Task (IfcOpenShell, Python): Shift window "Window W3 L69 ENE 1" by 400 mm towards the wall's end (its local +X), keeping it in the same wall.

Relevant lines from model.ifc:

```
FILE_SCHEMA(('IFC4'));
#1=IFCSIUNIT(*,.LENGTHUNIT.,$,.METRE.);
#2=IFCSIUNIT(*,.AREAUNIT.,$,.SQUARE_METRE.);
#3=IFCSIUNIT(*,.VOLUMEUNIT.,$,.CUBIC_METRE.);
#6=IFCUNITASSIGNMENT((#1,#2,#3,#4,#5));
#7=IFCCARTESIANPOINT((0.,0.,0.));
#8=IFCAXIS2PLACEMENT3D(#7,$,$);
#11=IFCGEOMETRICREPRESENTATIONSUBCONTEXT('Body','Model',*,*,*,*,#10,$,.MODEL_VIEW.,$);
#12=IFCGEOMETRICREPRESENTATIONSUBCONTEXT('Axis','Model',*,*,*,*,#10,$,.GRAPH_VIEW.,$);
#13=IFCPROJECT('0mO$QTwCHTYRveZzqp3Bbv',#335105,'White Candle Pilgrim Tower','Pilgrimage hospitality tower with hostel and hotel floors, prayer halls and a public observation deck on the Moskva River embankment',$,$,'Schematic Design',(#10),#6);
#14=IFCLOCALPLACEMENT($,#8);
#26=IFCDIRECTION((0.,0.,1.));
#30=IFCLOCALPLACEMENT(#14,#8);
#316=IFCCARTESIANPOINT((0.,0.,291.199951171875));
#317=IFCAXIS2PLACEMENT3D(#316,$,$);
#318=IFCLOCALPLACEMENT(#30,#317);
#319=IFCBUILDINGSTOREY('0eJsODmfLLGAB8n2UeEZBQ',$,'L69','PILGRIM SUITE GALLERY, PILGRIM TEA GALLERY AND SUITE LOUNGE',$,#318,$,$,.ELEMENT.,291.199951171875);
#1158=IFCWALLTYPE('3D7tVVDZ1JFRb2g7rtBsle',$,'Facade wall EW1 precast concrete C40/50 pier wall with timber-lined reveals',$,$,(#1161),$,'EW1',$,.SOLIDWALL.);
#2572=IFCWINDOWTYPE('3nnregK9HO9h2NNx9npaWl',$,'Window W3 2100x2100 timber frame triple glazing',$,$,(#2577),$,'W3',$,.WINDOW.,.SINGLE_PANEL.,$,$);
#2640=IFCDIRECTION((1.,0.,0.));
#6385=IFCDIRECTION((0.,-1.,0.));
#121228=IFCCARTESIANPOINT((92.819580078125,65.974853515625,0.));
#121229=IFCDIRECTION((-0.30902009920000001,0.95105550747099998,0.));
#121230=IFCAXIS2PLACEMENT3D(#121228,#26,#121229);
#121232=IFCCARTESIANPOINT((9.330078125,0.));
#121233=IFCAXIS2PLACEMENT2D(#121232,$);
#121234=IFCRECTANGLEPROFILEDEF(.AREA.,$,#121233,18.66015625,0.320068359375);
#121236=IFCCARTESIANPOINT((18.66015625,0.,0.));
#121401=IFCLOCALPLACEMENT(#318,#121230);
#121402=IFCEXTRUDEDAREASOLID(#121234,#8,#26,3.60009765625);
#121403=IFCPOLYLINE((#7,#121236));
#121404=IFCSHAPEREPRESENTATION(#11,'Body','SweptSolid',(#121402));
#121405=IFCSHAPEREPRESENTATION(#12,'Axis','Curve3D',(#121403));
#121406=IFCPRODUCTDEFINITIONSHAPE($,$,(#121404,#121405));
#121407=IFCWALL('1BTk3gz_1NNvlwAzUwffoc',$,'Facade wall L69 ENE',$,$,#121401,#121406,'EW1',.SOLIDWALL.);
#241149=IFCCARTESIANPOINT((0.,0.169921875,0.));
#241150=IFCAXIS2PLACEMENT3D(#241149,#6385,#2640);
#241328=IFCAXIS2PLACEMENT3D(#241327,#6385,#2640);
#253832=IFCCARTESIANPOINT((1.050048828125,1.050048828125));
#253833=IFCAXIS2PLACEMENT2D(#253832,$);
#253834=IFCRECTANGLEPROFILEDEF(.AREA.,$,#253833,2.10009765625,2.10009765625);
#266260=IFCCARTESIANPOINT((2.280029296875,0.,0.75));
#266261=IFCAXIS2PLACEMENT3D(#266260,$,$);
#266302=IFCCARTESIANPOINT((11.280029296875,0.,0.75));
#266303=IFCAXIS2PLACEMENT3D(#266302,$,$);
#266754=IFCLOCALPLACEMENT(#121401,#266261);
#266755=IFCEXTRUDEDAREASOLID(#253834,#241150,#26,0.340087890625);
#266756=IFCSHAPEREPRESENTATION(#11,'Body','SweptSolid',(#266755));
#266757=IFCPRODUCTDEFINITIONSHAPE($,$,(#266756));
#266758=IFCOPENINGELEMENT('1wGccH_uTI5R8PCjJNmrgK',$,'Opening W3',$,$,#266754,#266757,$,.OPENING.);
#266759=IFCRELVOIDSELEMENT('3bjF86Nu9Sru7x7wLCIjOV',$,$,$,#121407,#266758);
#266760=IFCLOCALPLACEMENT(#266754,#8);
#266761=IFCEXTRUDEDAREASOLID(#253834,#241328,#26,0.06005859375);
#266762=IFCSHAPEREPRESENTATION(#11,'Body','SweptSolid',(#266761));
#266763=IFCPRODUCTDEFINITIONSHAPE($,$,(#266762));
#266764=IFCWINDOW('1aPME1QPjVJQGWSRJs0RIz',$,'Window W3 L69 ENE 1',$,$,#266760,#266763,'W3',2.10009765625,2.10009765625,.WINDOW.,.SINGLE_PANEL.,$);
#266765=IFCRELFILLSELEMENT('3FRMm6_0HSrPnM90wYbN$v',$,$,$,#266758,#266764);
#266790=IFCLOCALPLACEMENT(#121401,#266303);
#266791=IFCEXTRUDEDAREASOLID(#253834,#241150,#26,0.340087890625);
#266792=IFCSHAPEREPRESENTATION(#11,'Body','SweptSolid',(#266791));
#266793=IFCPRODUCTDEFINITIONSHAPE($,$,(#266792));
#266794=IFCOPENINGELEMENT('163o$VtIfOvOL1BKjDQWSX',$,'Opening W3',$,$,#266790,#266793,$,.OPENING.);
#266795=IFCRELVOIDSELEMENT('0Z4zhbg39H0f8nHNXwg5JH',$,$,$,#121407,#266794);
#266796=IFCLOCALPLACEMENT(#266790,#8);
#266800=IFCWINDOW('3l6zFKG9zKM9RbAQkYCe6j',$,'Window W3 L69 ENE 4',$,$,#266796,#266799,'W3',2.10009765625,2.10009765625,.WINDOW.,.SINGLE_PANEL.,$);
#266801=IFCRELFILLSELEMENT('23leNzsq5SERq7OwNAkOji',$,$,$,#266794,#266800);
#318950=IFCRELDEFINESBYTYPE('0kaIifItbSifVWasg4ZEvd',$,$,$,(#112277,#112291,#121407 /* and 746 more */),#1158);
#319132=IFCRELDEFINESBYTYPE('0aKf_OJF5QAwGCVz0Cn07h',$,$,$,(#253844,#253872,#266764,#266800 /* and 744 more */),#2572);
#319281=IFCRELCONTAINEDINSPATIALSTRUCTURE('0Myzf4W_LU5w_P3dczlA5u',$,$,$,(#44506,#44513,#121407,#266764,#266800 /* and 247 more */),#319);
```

```python
import ifcopenshell
import ifcopenshell.api.geometry
import ifcopenshell.util.placement
import ifcopenshell.util.unit

model = ifcopenshell.open("model.ifc")
unit_scale = ifcopenshell.util.unit.calculate_unit_scale(model)

window = model.by_id(266764)
opening = window.FillsVoids[0].RelatingOpeningElement
wall = opening.VoidsElements[0].RelatingBuildingElement

wall_matrix = ifcopenshell.util.placement.get_local_placement(wall.ObjectPlacement)
shift = wall_matrix[:3, 0] * 0.4 / unit_scale
before = ifcopenshell.util.placement.get_local_placement(window.ObjectPlacement)[:3, 3].copy()

# The window is placed relative to its opening, so it follows when the opening moves.
matrix = ifcopenshell.util.placement.get_local_placement(opening.ObjectPlacement)
matrix[:3, 3] += shift
ifcopenshell.api.geometry.edit_object_placement(
    model, product=opening, matrix=matrix, is_si=False, should_transform_children=True
)

after = ifcopenshell.util.placement.get_local_placement(window.ObjectPlacement)[:3, 3]
print("window moved by", (after - before).round(3) + 0.0)

model.write("model_rev.ifc")
```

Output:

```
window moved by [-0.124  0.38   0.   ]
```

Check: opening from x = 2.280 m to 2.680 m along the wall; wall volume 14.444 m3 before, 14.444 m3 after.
